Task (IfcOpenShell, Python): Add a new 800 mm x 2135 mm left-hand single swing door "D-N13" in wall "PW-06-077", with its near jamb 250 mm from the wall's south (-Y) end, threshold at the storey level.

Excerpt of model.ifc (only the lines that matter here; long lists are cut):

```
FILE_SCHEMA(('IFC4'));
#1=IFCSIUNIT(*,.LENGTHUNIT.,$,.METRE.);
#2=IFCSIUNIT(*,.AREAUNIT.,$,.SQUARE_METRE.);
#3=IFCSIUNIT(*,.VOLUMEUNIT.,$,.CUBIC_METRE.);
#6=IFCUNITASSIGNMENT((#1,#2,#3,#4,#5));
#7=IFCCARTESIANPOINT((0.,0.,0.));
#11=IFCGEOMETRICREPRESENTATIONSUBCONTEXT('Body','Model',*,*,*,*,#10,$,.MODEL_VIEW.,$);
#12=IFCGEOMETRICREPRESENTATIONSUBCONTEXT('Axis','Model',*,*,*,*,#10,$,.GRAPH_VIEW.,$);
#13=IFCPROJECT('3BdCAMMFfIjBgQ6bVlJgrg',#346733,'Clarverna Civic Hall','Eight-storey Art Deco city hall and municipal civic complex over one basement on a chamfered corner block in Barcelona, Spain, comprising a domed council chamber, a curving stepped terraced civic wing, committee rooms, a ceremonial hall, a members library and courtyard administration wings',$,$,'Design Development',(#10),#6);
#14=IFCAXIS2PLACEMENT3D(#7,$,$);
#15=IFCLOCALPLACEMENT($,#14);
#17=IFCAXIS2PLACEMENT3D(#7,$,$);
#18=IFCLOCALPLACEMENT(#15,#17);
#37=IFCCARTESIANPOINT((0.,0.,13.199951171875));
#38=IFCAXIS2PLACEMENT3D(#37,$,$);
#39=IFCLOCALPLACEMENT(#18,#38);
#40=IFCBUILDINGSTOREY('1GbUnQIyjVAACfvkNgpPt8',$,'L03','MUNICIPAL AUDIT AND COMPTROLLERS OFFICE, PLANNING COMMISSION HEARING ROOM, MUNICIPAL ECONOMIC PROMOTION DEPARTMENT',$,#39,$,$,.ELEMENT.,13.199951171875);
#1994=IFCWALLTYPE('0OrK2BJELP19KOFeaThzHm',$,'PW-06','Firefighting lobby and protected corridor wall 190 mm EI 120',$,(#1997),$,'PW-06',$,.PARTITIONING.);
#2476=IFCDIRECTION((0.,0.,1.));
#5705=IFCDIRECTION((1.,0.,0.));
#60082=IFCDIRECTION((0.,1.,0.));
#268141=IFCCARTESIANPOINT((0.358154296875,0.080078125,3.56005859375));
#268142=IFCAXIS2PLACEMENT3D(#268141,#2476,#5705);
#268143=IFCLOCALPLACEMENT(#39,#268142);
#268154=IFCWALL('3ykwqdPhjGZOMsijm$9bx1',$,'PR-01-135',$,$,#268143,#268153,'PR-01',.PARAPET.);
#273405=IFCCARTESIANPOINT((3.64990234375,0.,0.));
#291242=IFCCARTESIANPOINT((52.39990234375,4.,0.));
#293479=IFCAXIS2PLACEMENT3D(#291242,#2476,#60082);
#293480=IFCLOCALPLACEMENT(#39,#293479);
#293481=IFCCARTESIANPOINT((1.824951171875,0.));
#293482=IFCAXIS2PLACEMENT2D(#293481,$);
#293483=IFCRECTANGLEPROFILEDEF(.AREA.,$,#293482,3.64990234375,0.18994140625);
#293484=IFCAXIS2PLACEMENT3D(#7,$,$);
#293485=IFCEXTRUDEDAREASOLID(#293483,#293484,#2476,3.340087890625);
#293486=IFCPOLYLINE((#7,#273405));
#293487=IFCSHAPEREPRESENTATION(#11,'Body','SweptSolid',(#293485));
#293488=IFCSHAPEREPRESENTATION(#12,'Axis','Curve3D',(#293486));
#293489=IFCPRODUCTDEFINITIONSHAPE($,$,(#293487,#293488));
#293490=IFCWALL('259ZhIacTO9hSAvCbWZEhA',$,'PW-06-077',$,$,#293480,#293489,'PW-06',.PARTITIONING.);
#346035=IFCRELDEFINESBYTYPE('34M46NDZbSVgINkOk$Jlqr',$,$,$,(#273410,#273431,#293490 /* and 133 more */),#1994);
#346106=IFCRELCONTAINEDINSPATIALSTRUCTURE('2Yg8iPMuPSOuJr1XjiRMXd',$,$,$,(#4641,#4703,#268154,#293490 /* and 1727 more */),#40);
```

```python
import numpy as np
import ifcopenshell
import ifcopenshell.api.feature
import ifcopenshell.api.geometry
import ifcopenshell.api.root
import ifcopenshell.api.spatial
import ifcopenshell.geom
import ifcopenshell.util.element
import ifcopenshell.util.placement
import ifcopenshell.util.representation
import ifcopenshell.util.shape
import ifcopenshell.util.unit

model = ifcopenshell.open("model.ifc")
unit_scale = ifcopenshell.util.unit.calculate_unit_scale(model)
settings = ifcopenshell.geom.settings()


def volume(element):
    """Net volume in cubic metres, openings subtracted."""
    shape = ifcopenshell.geom.create_shape(settings, element)
    return ifcopenshell.util.shape.get_volume(shape.geometry)


wall = model.by_guid("259ZhIacTO9hSAvCbWZEhA")
storey = ifcopenshell.util.element.get_container(wall, ifc_class="IfcBuildingStorey")
context = ifcopenshell.util.representation.get_context(model, "Model", "Body", "MODEL_VIEW")
before = volume(wall)

width, height, from_end, sill = 0.8, 2.135, 0.25, 0.0  # metres

# The wall runs along its own X axis, and the end named is its -X end.
wall_shape = ifcopenshell.geom.create_shape(settings, wall)
x, y, z = ifcopenshell.util.shape.get_vertices(wall_shape.geometry).T
start = x.min() + from_end
face, thickness = float(y.min()), float(y.max() - y.min())
wall_matrix = ifcopenshell.util.placement.get_local_placement(wall.ObjectPlacement)
level = ifcopenshell.util.placement.get_local_placement(storey.ObjectPlacement)[2, 3]


def in_wall(x, y):
    """Placement at x, y metres in the wall's axes, at sill height."""
    matrix = wall_matrix.copy()
    matrix[:, 3] = wall_matrix @ np.array([x / unit_scale, y / unit_scale, 0.0, 1.0])
    matrix[2, 3] = level + sill / unit_scale
    return matrix


# Opening: a box that overshoots both wall faces by 50 mm.
opening = ifcopenshell.api.root.create_entity(model, ifc_class="IfcOpeningElement", predefined_type="OPENING")
box = ifcopenshell.api.geometry.add_wall_representation(
    model, context=context, length=width, height=height, thickness=thickness + 0.1
)
ifcopenshell.api.geometry.assign_representation(model, product=opening, representation=box)
ifcopenshell.api.geometry.edit_object_placement(model, product=opening, matrix=in_wall(start, face - 0.05), is_si=False)
ifcopenshell.api.feature.add_feature(model, feature=opening, element=wall)

door = ifcopenshell.api.root.create_entity(model, ifc_class="IfcDoor", name="D-N13", predefined_type="DOOR")
door.OverallWidth, door.OverallHeight = width / unit_scale, height / unit_scale
door.OperationType = "SINGLE_SWING_LEFT"
body = ifcopenshell.api.geometry.add_door_representation(
    model,
    context=context,
    overall_width=door.OverallWidth,
    overall_height=door.OverallHeight,
    operation_type="SINGLE_SWING_LEFT",
    lining_properties={"LiningDepth": thickness / unit_scale, "ThresholdDepth": thickness / unit_scale},
)
ifcopenshell.api.geometry.assign_representation(model, product=door, representation=body)
ifcopenshell.api.spatial.assign_container(model, products=[door], relating_structure=storey)
ifcopenshell.api.feature.add_filling(model, opening=opening, element=door)

# The lining spans the wall, so the door starts at the wall face.
ifcopenshell.api.geometry.edit_object_placement(model, product=door, matrix=in_wall(start, face), is_si=False)

after = volume(wall)

print(f"wall volume {before:.3f} -> {after:.3f} m3")

model.write("model_updated.ifc")
```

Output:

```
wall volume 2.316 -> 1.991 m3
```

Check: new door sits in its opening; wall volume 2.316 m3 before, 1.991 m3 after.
